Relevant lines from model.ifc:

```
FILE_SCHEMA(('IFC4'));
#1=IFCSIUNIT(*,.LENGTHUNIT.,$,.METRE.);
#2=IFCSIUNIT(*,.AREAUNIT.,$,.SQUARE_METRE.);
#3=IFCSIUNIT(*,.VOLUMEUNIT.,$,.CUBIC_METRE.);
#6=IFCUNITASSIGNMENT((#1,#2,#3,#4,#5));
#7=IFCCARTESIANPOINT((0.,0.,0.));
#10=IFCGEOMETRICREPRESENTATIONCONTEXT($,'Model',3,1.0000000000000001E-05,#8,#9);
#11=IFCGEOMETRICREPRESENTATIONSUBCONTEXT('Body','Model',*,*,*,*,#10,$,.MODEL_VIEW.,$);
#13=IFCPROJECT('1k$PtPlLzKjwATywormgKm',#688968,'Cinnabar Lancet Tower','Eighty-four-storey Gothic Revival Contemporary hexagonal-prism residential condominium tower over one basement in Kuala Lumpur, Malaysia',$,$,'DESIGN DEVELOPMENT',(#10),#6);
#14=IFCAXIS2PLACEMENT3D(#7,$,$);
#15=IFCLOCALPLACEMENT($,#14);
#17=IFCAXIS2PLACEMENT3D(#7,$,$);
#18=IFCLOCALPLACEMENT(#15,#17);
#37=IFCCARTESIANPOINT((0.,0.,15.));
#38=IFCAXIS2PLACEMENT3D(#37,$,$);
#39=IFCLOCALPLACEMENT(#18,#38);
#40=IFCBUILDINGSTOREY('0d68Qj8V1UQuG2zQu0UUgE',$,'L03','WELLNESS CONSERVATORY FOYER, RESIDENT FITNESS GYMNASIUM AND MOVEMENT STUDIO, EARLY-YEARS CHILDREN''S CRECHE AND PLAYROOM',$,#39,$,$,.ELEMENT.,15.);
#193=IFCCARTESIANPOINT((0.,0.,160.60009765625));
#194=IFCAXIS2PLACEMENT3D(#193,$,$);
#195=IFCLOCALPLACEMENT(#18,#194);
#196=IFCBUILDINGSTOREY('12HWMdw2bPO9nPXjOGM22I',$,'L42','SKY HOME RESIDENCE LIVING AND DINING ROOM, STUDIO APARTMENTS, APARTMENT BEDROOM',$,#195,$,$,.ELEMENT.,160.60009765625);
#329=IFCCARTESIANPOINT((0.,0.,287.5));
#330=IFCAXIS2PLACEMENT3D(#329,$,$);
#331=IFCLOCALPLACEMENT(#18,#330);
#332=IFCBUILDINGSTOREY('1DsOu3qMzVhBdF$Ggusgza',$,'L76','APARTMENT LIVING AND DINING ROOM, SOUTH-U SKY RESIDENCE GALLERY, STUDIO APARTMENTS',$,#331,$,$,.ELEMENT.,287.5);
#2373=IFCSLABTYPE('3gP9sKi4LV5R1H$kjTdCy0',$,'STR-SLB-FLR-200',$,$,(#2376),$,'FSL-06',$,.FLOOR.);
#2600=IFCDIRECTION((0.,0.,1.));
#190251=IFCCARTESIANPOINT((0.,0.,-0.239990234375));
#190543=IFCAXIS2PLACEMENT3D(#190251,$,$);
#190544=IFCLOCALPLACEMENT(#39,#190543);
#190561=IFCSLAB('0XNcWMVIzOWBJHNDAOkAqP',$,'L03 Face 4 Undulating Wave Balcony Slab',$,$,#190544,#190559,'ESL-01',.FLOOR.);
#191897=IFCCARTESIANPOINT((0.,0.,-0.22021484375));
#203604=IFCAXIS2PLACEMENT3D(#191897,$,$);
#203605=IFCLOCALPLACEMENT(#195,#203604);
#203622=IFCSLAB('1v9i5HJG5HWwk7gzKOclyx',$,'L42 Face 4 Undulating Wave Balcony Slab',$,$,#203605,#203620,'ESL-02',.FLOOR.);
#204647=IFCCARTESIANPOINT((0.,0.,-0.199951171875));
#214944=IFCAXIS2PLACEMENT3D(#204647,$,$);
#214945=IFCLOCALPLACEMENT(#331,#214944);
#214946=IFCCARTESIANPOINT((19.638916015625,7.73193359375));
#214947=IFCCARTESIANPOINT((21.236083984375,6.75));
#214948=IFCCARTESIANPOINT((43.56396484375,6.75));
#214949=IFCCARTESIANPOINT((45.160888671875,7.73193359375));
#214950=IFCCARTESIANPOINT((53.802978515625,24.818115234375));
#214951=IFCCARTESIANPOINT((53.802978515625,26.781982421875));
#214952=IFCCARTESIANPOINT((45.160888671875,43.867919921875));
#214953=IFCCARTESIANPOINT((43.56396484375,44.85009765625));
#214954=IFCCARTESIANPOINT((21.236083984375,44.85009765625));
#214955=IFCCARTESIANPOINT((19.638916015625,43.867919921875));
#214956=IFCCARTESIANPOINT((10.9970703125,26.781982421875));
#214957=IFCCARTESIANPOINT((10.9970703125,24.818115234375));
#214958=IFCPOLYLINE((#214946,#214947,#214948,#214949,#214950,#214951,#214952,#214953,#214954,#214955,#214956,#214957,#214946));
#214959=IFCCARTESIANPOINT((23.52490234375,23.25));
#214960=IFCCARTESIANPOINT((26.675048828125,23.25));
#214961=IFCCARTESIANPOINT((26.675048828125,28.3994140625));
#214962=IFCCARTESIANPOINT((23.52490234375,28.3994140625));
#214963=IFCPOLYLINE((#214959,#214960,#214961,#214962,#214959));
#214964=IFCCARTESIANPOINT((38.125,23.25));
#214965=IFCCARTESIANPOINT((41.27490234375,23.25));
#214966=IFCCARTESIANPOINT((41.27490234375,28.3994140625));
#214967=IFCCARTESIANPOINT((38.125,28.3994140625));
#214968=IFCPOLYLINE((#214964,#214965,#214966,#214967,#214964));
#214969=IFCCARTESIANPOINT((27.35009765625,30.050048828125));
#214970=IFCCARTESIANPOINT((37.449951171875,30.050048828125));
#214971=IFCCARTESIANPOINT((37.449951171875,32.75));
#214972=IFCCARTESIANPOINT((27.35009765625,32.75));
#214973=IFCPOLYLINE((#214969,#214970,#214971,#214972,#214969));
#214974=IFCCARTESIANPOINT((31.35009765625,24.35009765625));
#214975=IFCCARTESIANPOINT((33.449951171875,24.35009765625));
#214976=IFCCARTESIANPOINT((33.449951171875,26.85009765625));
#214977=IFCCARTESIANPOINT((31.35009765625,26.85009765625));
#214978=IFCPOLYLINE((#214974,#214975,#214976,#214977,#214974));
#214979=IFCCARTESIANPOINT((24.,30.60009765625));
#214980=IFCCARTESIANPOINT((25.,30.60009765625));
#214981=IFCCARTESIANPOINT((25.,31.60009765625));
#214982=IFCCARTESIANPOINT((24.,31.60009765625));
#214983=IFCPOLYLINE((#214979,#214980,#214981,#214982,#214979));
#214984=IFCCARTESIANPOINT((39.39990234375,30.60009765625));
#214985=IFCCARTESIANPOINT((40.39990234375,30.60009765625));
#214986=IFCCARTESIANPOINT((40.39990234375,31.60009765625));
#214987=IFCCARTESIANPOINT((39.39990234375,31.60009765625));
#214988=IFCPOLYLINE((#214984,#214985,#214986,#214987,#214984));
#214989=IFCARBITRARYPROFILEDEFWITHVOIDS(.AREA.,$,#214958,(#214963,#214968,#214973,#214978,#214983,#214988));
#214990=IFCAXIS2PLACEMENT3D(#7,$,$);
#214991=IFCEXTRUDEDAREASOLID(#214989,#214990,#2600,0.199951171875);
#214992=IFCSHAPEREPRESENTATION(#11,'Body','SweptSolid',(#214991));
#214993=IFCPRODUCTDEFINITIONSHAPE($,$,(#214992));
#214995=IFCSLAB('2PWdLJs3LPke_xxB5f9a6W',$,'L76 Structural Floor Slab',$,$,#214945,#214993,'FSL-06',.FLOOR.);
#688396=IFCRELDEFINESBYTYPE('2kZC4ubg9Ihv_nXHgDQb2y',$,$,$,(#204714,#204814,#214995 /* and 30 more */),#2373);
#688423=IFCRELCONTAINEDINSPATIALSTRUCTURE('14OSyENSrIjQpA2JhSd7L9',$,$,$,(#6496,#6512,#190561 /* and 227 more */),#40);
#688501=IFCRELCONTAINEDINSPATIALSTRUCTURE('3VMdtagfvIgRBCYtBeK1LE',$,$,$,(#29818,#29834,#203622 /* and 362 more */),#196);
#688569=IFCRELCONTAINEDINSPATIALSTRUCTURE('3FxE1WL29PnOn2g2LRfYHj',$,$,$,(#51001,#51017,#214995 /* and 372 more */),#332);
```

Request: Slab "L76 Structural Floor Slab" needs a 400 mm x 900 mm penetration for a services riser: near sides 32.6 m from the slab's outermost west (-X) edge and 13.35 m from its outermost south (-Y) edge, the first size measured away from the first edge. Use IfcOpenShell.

```python
import numpy as np
import ifcopenshell
import ifcopenshell.api.feature
import ifcopenshell.api.geometry
import ifcopenshell.api.root
import ifcopenshell.geom
import ifcopenshell.util.placement
import ifcopenshell.util.representation
import ifcopenshell.util.shape
import ifcopenshell.util.unit

model = ifcopenshell.open("model.ifc")
unit_scale = ifcopenshell.util.unit.calculate_unit_scale(model)
settings = ifcopenshell.geom.settings()


def volume(element):
    """Net volume in cubic metres, openings subtracted."""
    shape = ifcopenshell.geom.create_shape(settings, element)
    return ifcopenshell.util.shape.get_volume(shape.geometry)


slab = model.by_guid("2PWdLJs3LPke_xxB5f9a6W")
before = volume(slab)

# Extent in the slab's own axes, in metres. The edges named are its -X and -Y sides.
slab_shape = ifcopenshell.geom.create_shape(settings, slab)
vertices = ifcopenshell.util.shape.get_vertices(slab_shape.geometry)
x_min, y_min, bottom = vertices.min(axis=0)
top = vertices[:, 2].max()

opening = ifcopenshell.api.root.create_entity(model, ifc_class="IfcOpeningElement", name="Services riser opening", predefined_type="OPENING")
context = ifcopenshell.util.representation.get_context(model, "Model", "Body", "MODEL_VIEW")
width, depth = 0.4, 0.9
outline = [(0.0, 0.0), (width, 0.0), (width, depth), (0.0, depth), (0.0, 0.0)]
# Overshoot both faces by 50 mm so the cut is clean.
shape = ifcopenshell.api.geometry.add_slab_representation(
    model, context=context, depth=top - bottom + 0.1, polyline=outline
)
ifcopenshell.api.geometry.assign_representation(model, product=opening, representation=shape)

matrix = ifcopenshell.util.placement.get_local_placement(slab.ObjectPlacement)
matrix[:, 3] = matrix @ np.append(np.array([x_min + 32.6, y_min + 13.35, bottom - 0.05]) / unit_scale, 1.0)
ifcopenshell.api.geometry.edit_object_placement(model, product=opening, matrix=matrix, is_si=False)
ifcopenshell.api.feature.add_feature(model, feature=opening, element=slab)

after = volume(slab)

print(f"slab volume {before:.3f} -> {after:.3f} m3")

model.write("model_updated.ifc")
```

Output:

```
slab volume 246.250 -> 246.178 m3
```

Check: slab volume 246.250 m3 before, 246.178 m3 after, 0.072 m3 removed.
